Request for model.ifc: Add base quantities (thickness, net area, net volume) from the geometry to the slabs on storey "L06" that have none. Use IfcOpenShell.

First a look at what the model holds.

```python
import ifcopenshell
import ifcopenshell.util.element
import ifcopenshell.util.unit

model = ifcopenshell.open("model.ifc")
print(model.schema)
for unit_type in ("LENGTHUNIT", "AREAUNIT", "VOLUMEUNIT"):
    print(unit_type, ifcopenshell.util.unit.calculate_unit_scale(model, unit_type))
storey = next(s for s in model.by_type("IfcBuildingStorey") if s.Name == "L06")
slabs = [e for e in ifcopenshell.util.element.get_decomposition(storey) if e.is_a("IfcSlab")]
for e in sorted(slabs, key=lambda e: e.id()):
    print(e.id(), e.is_a(), e.Name, list(ifcopenshell.util.element.get_psets(e, qtos_only=True)), sep=" | ")
```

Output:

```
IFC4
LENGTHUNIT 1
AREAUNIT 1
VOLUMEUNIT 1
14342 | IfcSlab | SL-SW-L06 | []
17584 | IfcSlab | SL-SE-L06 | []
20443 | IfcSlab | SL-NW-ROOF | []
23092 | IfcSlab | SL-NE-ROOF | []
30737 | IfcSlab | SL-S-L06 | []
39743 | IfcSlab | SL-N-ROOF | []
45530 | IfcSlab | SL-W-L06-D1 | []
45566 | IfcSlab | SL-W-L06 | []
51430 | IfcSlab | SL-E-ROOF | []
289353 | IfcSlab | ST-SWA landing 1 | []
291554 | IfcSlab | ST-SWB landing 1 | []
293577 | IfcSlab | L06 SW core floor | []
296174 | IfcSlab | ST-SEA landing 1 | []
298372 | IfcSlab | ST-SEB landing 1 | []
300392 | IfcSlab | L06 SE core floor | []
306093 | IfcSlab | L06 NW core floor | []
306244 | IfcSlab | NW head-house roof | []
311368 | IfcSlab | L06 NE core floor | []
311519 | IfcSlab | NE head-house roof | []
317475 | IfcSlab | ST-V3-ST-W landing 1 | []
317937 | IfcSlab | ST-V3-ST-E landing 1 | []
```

```python
import ifcopenshell
import ifcopenshell.api.pset
import ifcopenshell.geom
import ifcopenshell.util.element
import ifcopenshell.util.shape
import ifcopenshell.util.unit

model = ifcopenshell.open("model.ifc")
unit_scale = ifcopenshell.util.unit.calculate_unit_scale(model)
area_scale = ifcopenshell.util.unit.calculate_unit_scale(model, "AREAUNIT")
volume_scale = ifcopenshell.util.unit.calculate_unit_scale(model, "VOLUMEUNIT")
settings = ifcopenshell.geom.settings()

storey = next(s for s in model.by_type("IfcBuildingStorey") if s.Name == "L06")
slabs = [e for e in ifcopenshell.util.element.get_decomposition(storey) if e.is_a("IfcSlab")]

for e in sorted(slabs, key=lambda e: e.id()):
    if ifcopenshell.util.element.get_psets(e, qtos_only=True, should_inherit=False):
        continue
    # Geometry comes back in metres, in the element's own axes.
    shape = ifcopenshell.geom.create_shape(settings, e)
    values = {
        "Width": ifcopenshell.util.shape.get_z(shape.geometry) / unit_scale,
        "NetArea": ifcopenshell.util.shape.get_footprint_area(shape.geometry) / area_scale,
        "NetVolume": ifcopenshell.util.shape.get_volume(shape.geometry) / volume_scale,
    }
    qto = ifcopenshell.api.pset.add_qto(model, product=e, name="Qto_SlabBaseQuantities")
    ifcopenshell.api.pset.edit_qto(model, qto=qto, properties=values)
    print(e.id(), {k: round(v, 3) for k, v in values.items()})

model.write("model_rev.ifc")
```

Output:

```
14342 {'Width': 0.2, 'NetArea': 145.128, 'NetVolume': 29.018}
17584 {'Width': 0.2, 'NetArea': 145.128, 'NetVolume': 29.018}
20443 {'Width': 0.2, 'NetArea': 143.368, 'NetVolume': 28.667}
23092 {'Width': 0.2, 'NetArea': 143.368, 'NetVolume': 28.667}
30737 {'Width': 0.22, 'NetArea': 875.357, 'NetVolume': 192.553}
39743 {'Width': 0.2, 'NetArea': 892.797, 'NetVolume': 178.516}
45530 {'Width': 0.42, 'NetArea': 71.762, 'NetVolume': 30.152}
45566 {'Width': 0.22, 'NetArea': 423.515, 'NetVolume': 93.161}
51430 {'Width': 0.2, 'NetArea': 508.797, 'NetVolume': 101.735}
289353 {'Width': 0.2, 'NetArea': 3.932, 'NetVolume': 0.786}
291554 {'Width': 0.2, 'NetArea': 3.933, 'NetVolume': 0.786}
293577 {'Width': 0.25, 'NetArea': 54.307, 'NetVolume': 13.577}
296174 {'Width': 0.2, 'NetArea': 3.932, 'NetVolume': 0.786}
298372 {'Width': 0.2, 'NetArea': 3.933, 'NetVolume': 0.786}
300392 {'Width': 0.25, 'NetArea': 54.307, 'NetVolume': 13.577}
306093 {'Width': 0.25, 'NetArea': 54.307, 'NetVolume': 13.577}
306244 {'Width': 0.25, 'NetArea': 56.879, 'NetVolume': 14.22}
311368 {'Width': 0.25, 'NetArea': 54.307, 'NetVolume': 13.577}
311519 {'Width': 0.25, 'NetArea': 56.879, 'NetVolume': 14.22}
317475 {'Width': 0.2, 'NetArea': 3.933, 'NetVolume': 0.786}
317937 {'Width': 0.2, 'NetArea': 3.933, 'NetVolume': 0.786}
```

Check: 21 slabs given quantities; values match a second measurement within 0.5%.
